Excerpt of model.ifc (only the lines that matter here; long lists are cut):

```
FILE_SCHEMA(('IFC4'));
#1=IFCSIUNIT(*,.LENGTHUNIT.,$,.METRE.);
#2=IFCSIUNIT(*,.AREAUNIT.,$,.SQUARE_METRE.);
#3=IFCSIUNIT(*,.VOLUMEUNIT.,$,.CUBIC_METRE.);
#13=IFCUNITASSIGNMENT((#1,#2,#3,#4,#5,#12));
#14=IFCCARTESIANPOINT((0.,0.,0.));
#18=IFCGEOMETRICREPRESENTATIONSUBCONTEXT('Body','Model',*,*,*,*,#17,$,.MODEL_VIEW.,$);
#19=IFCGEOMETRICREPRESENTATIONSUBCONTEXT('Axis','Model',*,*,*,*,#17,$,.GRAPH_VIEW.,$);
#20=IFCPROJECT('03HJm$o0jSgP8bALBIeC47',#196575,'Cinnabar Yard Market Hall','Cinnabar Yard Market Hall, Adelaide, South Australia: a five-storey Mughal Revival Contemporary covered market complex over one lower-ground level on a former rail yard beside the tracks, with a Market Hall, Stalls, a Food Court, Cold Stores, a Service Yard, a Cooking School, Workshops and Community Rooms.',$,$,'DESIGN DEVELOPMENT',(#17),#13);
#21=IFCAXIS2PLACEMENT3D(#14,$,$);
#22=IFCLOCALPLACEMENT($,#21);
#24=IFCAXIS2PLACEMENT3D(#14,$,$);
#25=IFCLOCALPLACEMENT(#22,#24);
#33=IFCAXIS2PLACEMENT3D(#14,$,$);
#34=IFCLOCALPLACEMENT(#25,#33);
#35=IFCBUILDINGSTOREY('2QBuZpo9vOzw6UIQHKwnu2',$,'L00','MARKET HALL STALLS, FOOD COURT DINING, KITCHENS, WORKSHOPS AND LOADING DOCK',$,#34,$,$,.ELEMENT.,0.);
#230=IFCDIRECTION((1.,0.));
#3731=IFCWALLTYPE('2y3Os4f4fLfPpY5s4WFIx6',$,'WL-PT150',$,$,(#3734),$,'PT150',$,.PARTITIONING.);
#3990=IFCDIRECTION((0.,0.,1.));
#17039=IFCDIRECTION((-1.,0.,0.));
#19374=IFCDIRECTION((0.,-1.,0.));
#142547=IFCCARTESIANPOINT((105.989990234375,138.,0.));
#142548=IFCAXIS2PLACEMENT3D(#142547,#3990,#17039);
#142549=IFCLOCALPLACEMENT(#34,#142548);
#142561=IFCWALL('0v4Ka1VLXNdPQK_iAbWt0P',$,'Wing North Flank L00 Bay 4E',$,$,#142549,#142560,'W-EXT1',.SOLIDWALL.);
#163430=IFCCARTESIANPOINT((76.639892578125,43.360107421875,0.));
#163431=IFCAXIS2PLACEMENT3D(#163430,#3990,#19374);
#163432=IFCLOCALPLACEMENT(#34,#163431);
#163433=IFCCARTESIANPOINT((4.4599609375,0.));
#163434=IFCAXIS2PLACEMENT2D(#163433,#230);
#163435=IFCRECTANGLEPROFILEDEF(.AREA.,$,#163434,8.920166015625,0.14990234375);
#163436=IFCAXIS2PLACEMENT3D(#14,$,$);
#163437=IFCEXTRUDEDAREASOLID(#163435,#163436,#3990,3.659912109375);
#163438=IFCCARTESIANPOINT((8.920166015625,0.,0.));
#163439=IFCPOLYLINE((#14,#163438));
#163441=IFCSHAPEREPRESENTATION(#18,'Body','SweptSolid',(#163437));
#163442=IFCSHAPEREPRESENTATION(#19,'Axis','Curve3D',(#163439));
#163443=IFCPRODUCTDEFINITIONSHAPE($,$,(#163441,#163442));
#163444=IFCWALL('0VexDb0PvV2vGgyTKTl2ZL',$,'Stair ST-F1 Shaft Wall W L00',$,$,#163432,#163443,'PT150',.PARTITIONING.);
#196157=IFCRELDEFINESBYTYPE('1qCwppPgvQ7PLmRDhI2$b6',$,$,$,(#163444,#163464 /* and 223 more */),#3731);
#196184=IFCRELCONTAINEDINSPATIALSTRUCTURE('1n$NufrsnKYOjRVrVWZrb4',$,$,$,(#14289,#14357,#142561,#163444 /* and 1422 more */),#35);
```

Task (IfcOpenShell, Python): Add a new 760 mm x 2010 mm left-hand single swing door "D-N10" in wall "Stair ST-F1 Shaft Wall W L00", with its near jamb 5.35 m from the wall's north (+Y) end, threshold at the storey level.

```python
import numpy as np
import ifcopenshell
import ifcopenshell.api.feature
import ifcopenshell.api.geometry
import ifcopenshell.api.root
import ifcopenshell.api.spatial
import ifcopenshell.geom
import ifcopenshell.util.element
import ifcopenshell.util.placement
import ifcopenshell.util.representation
import ifcopenshell.util.shape
import ifcopenshell.util.unit

model = ifcopenshell.open("model.ifc")
unit_scale = ifcopenshell.util.unit.calculate_unit_scale(model)
settings = ifcopenshell.geom.settings()


def volume(element):
    """Net volume in cubic metres, openings subtracted."""
    shape = ifcopenshell.geom.create_shape(settings, element)
    return ifcopenshell.util.shape.get_volume(shape.geometry)


wall = model.by_guid("0VexDb0PvV2vGgyTKTl2ZL")
storey = ifcopenshell.util.element.get_container(wall, ifc_class="IfcBuildingStorey")
context = ifcopenshell.util.representation.get_context(model, "Model", "Body", "MODEL_VIEW")
before = volume(wall)

width, height, from_end, sill = 0.76, 2.01, 5.35, 0.0  # metres

# The wall runs along its own X axis, and the end named is its -X end.
wall_shape = ifcopenshell.geom.create_shape(settings, wall)
x, y, z = ifcopenshell.util.shape.get_vertices(wall_shape.geometry).T
start = x.min() + from_end
face, thickness = float(y.min()), float(y.max() - y.min())
wall_matrix = ifcopenshell.util.placement.get_local_placement(wall.ObjectPlacement)
level = ifcopenshell.util.placement.get_local_placement(storey.ObjectPlacement)[2, 3]


def in_wall(x, y):
    """Placement at x, y metres in the wall's axes, at sill height."""
    matrix = wall_matrix.copy()
    matrix[:, 3] = wall_matrix @ np.array([x / unit_scale, y / unit_scale, 0.0, 1.0])
    matrix[2, 3] = level + sill / unit_scale
    return matrix


# Opening: a box that overshoots both wall faces by 50 mm.
opening = ifcopenshell.api.root.create_entity(model, ifc_class="IfcOpeningElement", predefined_type="OPENING")
box = ifcopenshell.api.geometry.add_wall_representation(
    model, context=context, length=width, height=height, thickness=thickness + 0.1
)
ifcopenshell.api.geometry.assign_representation(model, product=opening, representation=box)
ifcopenshell.api.geometry.edit_object_placement(model, product=opening, matrix=in_wall(start, face - 0.05), is_si=False)
ifcopenshell.api.feature.add_feature(model, feature=opening, element=wall)

door = ifcopenshell.api.root.create_entity(model, ifc_class="IfcDoor", name="D-N10", predefined_type="DOOR")
door.OverallWidth, door.OverallHeight = width / unit_scale, height / unit_scale
door.OperationType = "SINGLE_SWING_LEFT"
body = ifcopenshell.api.geometry.add_door_representation(
    model,
    context=context,
    overall_width=door.OverallWidth,
    overall_height=door.OverallHeight,
    operation_type="SINGLE_SWING_LEFT",
    lining_properties={"LiningDepth": thickness / unit_scale, "ThresholdDepth": thickness / unit_scale},
)
ifcopenshell.api.geometry.assign_representation(model, product=door, representation=body)
ifcopenshell.api.spatial.assign_container(model, products=[door], relating_structure=storey)
ifcopenshell.api.feature.add_filling(model, opening=opening, element=door)

# The lining spans the wall, so the door starts at the wall face.
ifcopenshell.api.geometry.edit_object_placement(model, product=door, matrix=in_wall(start, face), is_si=False)

after = volume(wall)

print(f"wall volume {before:.3f} -> {after:.3f} m3")

model.write("model-out.ifc")
```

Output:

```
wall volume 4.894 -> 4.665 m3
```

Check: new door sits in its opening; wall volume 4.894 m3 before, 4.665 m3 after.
